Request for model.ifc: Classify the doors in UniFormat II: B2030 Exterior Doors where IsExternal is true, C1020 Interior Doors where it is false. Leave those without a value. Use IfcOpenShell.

First a look at what the model holds.

```python
import ifcopenshell
import ifcopenshell.util.element

model = ifcopenshell.open("model.ifc")
print(model.schema)
print("classifications:", [c.Name for c in model.by_type("IfcClassification")])
values = [ifcopenshell.util.element.get_pset(e, "Pset_DoorCommon", "IsExternal") for e in model.by_type("IfcDoor")]
for value in (True, False, None):
    print("IsExternal", value, values.count(value))
```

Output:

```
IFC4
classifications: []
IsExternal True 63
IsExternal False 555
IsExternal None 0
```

```python
import ifcopenshell
import ifcopenshell.api.classification
import ifcopenshell.util.element

model = ifcopenshell.open("model.ifc")

system = ifcopenshell.api.classification.add_classification(model, classification="UniFormat II")

doors = model.by_type("IfcDoor")
external = {e: ifcopenshell.util.element.get_pset(e, "Pset_DoorCommon", "IsExternal") for e in doors}
for flag, code, name in ((True, "B2030", "Exterior Doors"), (False, "C1020", "Interior Doors")):
    products = [e for e in doors if external[e] is flag]
    ifcopenshell.api.classification.add_reference(
        model, products=products, classification=system, identification=code, name=name
    )
    print(code, len(products))

model.write("model-out.ifc")
```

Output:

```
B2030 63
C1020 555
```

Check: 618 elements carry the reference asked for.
